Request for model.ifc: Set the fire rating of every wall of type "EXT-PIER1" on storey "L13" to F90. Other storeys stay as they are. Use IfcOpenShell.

First a look at what the model holds.

```python
import ifcopenshell
import ifcopenshell.util.element

model = ifcopenshell.open("model.ifc")
print(model.schema)
storey = next(s for s in model.by_type("IfcBuildingStorey") if s.Name == "L13")
walls = [e for e in ifcopenshell.util.element.get_decomposition(storey) if e.is_a("IfcWall")]
seen = {}
for e in walls:
    element_type = ifcopenshell.util.element.get_type(e)
    key = (element_type.Name if element_type != e and element_type else None, ifcopenshell.util.element.get_pset(e, "Pset_WallCommon", "FireRating"))
    seen[key] = seen.get(key, 0) + 1
for (name, value), count in sorted(seen.items(), key=str):
    print(count, "x", name, "|", value)
```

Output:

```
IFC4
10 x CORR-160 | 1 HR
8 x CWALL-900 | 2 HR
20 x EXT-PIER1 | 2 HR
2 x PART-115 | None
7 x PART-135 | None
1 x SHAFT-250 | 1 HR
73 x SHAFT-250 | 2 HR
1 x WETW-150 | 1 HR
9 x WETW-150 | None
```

```python
import ifcopenshell
import ifcopenshell.api.pset
import ifcopenshell.util.element

model = ifcopenshell.open("model.ifc")

storey = next(s for s in model.by_type("IfcBuildingStorey") if s.Name == "L13")
walls = [e for e in ifcopenshell.util.element.get_decomposition(storey) if e.is_a("IfcWall")]

count = 0
for e in walls:
    element_type = ifcopenshell.util.element.get_type(e)
    if element_type in (None, e) or element_type.Name != "EXT-PIER1":
        continue
    # add_pset returns the element's existing set when there is one.
    pset = ifcopenshell.api.pset.add_pset(model, product=e, name="Pset_WallCommon")
    ifcopenshell.api.pset.edit_pset(model, pset=pset, properties={"FireRating": "F90"})
    count += 1

print(count, "walls updated")

model.write("model_v2.ifc")
```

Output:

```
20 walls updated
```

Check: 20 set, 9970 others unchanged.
